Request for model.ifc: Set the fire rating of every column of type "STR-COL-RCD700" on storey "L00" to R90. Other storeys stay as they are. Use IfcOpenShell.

First a look at what the model holds.

```python
import ifcopenshell
import ifcopenshell.util.element

model = ifcopenshell.open("model.ifc")
print(model.schema)
storey = next(s for s in model.by_type("IfcBuildingStorey") if s.Name == "L00")
columns = [e for e in ifcopenshell.util.element.get_decomposition(storey) if e.is_a("IfcColumn")]
seen = {}
for e in columns:
    element_type = ifcopenshell.util.element.get_type(e)
    key = (element_type.Name if element_type != e and element_type else None, ifcopenshell.util.element.get_pset(e, "Pset_ColumnCommon", "FireRating"))
    seen[key] = seen.get(key, 0) + 1
for (name, value), count in sorted(seen.items(), key=str):
    print(count, "x", name, "|", value)
```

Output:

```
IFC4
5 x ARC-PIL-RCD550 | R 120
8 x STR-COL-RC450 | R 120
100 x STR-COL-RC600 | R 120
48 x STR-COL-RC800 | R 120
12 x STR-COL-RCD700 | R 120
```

```python
import ifcopenshell
import ifcopenshell.api.pset
import ifcopenshell.util.element

model = ifcopenshell.open("model.ifc")

storey = next(s for s in model.by_type("IfcBuildingStorey") if s.Name == "L00")
columns = [e for e in ifcopenshell.util.element.get_decomposition(storey) if e.is_a("IfcColumn")]

count = 0
for e in columns:
    element_type = ifcopenshell.util.element.get_type(e)
    if element_type in (None, e) or element_type.Name != "STR-COL-RCD700":
        continue
    # add_pset returns the element's existing set when there is one.
    pset = ifcopenshell.api.pset.add_pset(model, product=e, name="Pset_ColumnCommon")
    ifcopenshell.api.pset.edit_pset(model, pset=pset, properties={"FireRating": "R90"})
    count += 1

print(count, "columns updated")

model.write("model_v2.ifc")
```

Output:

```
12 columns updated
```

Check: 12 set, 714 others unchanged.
